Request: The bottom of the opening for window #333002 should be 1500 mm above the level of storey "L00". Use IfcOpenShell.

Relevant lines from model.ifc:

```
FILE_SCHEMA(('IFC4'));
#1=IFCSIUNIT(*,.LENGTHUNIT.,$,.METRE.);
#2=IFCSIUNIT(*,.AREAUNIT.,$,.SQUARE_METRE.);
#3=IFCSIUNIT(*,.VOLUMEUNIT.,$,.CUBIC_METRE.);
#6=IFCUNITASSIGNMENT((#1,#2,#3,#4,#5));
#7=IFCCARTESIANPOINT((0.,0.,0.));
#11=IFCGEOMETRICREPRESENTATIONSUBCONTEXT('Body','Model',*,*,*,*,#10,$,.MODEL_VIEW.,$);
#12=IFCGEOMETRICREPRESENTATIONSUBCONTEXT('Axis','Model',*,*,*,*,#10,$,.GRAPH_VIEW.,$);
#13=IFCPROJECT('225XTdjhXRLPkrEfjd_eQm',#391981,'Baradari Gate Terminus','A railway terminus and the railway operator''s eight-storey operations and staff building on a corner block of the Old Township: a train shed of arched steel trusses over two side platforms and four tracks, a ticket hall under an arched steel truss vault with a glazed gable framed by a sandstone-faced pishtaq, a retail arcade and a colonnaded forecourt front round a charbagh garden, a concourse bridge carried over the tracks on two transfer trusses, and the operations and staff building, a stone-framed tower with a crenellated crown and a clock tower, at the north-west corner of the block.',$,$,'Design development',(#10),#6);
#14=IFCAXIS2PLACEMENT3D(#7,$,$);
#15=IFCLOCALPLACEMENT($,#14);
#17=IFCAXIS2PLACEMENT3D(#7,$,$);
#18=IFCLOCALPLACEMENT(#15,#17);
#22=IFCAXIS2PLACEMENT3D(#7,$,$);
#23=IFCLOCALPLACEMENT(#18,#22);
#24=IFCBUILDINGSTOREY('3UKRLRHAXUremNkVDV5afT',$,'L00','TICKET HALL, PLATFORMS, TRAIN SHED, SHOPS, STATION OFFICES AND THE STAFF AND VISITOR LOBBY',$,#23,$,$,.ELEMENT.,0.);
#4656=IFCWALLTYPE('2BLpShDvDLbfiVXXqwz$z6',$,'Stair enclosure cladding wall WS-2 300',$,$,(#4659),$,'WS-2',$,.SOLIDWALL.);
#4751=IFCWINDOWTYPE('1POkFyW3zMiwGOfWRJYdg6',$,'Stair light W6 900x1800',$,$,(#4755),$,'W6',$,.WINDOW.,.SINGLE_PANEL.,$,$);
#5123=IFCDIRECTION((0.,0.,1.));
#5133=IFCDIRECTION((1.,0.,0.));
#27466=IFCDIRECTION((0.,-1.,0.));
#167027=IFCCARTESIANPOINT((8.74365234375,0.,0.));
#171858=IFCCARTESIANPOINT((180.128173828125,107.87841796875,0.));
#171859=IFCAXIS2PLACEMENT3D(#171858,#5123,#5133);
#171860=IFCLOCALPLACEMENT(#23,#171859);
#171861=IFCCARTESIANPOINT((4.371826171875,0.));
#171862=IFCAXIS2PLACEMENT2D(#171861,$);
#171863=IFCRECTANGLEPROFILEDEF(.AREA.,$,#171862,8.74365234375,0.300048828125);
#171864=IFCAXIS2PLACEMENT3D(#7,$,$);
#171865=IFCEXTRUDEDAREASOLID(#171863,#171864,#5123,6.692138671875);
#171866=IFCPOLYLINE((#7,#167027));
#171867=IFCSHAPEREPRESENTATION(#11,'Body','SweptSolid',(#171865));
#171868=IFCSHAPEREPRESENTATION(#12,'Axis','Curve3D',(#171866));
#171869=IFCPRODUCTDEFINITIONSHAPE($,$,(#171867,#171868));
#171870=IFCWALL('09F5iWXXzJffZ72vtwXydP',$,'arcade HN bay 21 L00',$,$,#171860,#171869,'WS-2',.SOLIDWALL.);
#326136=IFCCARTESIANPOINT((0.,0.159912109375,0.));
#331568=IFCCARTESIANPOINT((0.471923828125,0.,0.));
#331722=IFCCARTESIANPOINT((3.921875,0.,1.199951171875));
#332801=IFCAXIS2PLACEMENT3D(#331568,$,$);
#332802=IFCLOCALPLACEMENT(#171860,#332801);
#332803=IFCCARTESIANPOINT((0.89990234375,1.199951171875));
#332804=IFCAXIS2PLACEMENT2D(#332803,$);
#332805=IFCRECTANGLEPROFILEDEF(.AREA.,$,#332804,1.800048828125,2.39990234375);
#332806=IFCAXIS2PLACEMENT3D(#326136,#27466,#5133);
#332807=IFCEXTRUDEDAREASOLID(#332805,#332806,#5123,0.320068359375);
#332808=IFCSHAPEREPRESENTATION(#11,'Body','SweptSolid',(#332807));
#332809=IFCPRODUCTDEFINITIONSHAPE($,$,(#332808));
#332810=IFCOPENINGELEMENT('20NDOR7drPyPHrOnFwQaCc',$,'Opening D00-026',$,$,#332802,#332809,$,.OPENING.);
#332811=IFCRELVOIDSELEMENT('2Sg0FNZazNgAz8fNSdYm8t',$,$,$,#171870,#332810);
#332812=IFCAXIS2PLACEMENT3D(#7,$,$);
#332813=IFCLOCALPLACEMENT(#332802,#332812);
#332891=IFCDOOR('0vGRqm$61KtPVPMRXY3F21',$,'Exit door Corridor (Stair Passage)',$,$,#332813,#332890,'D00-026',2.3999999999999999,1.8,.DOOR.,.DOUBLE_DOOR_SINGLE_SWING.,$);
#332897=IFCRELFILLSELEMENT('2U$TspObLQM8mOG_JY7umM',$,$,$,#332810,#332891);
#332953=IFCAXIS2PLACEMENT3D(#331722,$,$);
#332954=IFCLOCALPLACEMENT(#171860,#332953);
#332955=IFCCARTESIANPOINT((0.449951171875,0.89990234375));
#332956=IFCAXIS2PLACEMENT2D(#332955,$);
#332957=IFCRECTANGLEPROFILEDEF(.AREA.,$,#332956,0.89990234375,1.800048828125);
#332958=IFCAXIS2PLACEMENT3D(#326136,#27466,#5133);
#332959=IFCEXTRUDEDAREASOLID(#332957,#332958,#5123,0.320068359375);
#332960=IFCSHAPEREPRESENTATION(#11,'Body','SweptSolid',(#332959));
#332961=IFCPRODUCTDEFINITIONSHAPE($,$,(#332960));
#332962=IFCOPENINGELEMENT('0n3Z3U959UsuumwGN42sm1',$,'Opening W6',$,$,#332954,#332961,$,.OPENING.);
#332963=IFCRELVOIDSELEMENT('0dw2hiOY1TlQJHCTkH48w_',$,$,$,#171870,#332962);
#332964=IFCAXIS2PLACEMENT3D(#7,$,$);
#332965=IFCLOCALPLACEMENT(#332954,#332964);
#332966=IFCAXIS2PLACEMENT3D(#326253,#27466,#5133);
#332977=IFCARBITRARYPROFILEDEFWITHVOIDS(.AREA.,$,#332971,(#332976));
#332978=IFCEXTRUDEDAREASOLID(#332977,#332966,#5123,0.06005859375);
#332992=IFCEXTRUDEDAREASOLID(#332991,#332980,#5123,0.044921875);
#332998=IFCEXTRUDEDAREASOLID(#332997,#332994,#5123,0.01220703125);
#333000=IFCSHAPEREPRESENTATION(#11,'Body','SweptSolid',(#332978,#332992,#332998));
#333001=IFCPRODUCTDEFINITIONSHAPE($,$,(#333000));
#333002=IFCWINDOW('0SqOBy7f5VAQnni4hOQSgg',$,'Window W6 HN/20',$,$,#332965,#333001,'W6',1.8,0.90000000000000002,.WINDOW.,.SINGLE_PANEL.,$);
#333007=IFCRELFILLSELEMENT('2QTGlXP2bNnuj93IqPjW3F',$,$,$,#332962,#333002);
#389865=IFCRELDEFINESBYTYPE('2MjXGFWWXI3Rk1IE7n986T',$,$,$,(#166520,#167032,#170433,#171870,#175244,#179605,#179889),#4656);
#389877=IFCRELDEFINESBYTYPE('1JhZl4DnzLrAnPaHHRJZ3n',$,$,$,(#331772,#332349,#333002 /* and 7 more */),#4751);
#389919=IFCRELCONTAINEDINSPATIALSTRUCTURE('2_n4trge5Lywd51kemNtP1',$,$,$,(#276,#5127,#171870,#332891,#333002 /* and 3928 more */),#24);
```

```python
import numpy as np
import ifcopenshell
import ifcopenshell.api.geometry
import ifcopenshell.geom
import ifcopenshell.util.element
import ifcopenshell.util.placement
import ifcopenshell.util.shape
import ifcopenshell.util.unit

model = ifcopenshell.open("model.ifc")
unit_scale = ifcopenshell.util.unit.calculate_unit_scale(model)

window = model.by_id(333002)
opening = window.FillsVoids[0].RelatingOpeningElement
storey = ifcopenshell.util.element.get_container(window, ifc_class="IfcBuildingStorey")
level = ifcopenshell.util.placement.get_local_placement(storey.ObjectPlacement)[2, 3]

# The opening's origin need not be at the sill, so measure its lowest point.
shape = ifcopenshell.geom.create_shape(ifcopenshell.geom.settings(), opening)
bottom = ifcopenshell.util.shape.get_shape_bottom_elevation(shape, shape.geometry) / unit_scale
dz = level + 1.5 / unit_scale - bottom

shift = np.array([0.0, 0.0, dz])
# The window is placed relative to its opening, so it follows when the opening moves.
matrix = ifcopenshell.util.placement.get_local_placement(opening.ObjectPlacement)
matrix[:3, 3] += shift
ifcopenshell.api.geometry.edit_object_placement(
    model, product=opening, matrix=matrix, is_si=False, should_transform_children=True
)

print(f"moved by {dz * unit_scale:+.3f} m")

model.write("model_v2.ifc")
```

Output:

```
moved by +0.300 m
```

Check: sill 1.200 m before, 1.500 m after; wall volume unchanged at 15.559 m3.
